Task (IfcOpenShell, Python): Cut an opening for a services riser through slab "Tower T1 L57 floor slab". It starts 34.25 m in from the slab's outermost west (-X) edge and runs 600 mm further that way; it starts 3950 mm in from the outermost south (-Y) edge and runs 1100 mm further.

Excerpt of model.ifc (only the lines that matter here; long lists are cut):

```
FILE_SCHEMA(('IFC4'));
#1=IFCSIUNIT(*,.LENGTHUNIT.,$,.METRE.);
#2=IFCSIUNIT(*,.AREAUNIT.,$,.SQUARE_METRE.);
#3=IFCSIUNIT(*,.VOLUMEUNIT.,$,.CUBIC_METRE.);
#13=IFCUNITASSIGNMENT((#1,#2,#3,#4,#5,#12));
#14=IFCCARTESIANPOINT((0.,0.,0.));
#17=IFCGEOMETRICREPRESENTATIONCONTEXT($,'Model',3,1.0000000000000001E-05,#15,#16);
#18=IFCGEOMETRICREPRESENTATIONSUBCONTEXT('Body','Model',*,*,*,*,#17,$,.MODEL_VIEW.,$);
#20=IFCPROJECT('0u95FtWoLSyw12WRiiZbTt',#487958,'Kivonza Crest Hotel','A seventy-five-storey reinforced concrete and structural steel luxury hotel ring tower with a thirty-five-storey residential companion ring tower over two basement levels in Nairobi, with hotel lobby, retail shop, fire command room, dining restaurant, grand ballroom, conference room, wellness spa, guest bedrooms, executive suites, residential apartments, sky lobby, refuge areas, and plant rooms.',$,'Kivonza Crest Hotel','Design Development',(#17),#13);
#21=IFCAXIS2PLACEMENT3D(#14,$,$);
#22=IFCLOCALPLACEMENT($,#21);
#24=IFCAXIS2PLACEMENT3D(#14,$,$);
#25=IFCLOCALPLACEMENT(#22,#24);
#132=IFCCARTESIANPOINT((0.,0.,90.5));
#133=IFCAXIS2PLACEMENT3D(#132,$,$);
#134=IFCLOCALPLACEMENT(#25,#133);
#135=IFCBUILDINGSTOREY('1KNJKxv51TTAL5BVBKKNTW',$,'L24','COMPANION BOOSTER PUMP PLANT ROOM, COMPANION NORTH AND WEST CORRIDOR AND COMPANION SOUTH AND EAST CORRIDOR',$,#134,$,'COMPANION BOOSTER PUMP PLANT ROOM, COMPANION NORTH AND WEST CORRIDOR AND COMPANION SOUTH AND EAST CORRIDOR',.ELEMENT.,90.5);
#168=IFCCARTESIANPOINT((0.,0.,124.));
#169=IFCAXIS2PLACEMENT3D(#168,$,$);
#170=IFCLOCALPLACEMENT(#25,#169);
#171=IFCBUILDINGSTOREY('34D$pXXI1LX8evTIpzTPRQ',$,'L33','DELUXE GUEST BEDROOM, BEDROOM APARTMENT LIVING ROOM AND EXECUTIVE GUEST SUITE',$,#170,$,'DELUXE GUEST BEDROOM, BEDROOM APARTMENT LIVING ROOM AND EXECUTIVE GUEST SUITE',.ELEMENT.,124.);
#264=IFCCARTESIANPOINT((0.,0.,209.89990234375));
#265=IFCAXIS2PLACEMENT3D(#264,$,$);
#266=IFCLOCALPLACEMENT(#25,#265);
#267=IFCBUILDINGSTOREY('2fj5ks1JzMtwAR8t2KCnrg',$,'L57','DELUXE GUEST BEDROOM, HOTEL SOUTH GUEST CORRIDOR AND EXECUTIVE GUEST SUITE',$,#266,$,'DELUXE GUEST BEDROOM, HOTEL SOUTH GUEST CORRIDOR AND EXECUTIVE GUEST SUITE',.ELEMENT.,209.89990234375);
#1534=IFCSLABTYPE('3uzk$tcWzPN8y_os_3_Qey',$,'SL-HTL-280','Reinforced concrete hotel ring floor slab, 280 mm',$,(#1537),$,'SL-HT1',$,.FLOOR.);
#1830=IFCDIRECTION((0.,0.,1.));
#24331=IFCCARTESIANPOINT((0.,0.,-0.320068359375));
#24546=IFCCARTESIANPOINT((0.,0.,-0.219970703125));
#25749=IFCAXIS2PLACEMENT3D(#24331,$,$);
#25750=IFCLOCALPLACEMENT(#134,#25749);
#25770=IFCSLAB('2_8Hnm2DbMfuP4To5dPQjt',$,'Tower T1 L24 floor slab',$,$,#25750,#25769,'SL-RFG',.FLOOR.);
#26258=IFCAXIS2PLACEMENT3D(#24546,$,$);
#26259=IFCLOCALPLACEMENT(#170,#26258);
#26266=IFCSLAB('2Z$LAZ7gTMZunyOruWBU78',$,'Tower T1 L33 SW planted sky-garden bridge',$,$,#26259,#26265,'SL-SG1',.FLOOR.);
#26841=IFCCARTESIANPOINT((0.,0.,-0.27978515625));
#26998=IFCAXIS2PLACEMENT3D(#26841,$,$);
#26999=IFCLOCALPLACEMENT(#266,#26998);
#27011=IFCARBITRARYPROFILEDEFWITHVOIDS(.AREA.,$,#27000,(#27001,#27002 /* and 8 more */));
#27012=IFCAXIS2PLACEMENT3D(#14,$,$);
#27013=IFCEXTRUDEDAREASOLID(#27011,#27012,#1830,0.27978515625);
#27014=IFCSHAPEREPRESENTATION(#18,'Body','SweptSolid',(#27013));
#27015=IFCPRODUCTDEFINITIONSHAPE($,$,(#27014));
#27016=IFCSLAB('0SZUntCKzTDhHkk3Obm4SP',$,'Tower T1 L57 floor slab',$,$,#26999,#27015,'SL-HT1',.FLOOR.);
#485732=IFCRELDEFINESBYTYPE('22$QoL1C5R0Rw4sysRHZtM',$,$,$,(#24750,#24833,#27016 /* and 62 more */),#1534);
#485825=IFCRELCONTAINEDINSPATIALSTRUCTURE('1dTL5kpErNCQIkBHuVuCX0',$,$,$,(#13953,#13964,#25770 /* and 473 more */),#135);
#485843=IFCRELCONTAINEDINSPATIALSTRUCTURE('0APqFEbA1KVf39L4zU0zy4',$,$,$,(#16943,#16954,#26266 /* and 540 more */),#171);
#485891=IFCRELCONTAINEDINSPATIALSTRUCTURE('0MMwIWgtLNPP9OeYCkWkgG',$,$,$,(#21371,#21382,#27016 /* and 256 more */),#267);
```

```python
import numpy as np
import ifcopenshell
import ifcopenshell.api.feature
import ifcopenshell.api.geometry
import ifcopenshell.api.root
import ifcopenshell.geom
import ifcopenshell.util.placement
import ifcopenshell.util.representation
import ifcopenshell.util.shape
import ifcopenshell.util.unit

model = ifcopenshell.open("model.ifc")
unit_scale = ifcopenshell.util.unit.calculate_unit_scale(model)
settings = ifcopenshell.geom.settings()


def volume(element):
    """Net volume in cubic metres, openings subtracted."""
    shape = ifcopenshell.geom.create_shape(settings, element)
    return ifcopenshell.util.shape.get_volume(shape.geometry)


slab = model.by_guid("0SZUntCKzTDhHkk3Obm4SP")
before = volume(slab)

# Extent in the slab's own axes, in metres. The edges named are its -X and -Y sides.
slab_shape = ifcopenshell.geom.create_shape(settings, slab)
vertices = ifcopenshell.util.shape.get_vertices(slab_shape.geometry)
x_min, y_min, bottom = vertices.min(axis=0)
top = vertices[:, 2].max()

opening = ifcopenshell.api.root.create_entity(model, ifc_class="IfcOpeningElement", name="Services riser opening", predefined_type="OPENING")
context = ifcopenshell.util.representation.get_context(model, "Model", "Body", "MODEL_VIEW")
width, depth = 0.6, 1.1
outline = [(0.0, 0.0), (width, 0.0), (width, depth), (0.0, depth), (0.0, 0.0)]
# Overshoot both faces by 50 mm so the cut is clean.
shape = ifcopenshell.api.geometry.add_slab_representation(
    model, context=context, depth=top - bottom + 0.1, polyline=outline
)
ifcopenshell.api.geometry.assign_representation(model, product=opening, representation=shape)

matrix = ifcopenshell.util.placement.get_local_placement(slab.ObjectPlacement)
matrix[:, 3] = matrix @ np.append(np.array([x_min + 34.25, y_min + 3.95, bottom - 0.05]) / unit_scale, 1.0)
ifcopenshell.api.geometry.edit_object_placement(model, product=opening, matrix=matrix, is_si=False)
ifcopenshell.api.feature.add_feature(model, feature=opening, element=slab)

after = volume(slab)

print(f"slab volume {before:.3f} -> {after:.3f} m3")

model.write("model_v2.ifc")
```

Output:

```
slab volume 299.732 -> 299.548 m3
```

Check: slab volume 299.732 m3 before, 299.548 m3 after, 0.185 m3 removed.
